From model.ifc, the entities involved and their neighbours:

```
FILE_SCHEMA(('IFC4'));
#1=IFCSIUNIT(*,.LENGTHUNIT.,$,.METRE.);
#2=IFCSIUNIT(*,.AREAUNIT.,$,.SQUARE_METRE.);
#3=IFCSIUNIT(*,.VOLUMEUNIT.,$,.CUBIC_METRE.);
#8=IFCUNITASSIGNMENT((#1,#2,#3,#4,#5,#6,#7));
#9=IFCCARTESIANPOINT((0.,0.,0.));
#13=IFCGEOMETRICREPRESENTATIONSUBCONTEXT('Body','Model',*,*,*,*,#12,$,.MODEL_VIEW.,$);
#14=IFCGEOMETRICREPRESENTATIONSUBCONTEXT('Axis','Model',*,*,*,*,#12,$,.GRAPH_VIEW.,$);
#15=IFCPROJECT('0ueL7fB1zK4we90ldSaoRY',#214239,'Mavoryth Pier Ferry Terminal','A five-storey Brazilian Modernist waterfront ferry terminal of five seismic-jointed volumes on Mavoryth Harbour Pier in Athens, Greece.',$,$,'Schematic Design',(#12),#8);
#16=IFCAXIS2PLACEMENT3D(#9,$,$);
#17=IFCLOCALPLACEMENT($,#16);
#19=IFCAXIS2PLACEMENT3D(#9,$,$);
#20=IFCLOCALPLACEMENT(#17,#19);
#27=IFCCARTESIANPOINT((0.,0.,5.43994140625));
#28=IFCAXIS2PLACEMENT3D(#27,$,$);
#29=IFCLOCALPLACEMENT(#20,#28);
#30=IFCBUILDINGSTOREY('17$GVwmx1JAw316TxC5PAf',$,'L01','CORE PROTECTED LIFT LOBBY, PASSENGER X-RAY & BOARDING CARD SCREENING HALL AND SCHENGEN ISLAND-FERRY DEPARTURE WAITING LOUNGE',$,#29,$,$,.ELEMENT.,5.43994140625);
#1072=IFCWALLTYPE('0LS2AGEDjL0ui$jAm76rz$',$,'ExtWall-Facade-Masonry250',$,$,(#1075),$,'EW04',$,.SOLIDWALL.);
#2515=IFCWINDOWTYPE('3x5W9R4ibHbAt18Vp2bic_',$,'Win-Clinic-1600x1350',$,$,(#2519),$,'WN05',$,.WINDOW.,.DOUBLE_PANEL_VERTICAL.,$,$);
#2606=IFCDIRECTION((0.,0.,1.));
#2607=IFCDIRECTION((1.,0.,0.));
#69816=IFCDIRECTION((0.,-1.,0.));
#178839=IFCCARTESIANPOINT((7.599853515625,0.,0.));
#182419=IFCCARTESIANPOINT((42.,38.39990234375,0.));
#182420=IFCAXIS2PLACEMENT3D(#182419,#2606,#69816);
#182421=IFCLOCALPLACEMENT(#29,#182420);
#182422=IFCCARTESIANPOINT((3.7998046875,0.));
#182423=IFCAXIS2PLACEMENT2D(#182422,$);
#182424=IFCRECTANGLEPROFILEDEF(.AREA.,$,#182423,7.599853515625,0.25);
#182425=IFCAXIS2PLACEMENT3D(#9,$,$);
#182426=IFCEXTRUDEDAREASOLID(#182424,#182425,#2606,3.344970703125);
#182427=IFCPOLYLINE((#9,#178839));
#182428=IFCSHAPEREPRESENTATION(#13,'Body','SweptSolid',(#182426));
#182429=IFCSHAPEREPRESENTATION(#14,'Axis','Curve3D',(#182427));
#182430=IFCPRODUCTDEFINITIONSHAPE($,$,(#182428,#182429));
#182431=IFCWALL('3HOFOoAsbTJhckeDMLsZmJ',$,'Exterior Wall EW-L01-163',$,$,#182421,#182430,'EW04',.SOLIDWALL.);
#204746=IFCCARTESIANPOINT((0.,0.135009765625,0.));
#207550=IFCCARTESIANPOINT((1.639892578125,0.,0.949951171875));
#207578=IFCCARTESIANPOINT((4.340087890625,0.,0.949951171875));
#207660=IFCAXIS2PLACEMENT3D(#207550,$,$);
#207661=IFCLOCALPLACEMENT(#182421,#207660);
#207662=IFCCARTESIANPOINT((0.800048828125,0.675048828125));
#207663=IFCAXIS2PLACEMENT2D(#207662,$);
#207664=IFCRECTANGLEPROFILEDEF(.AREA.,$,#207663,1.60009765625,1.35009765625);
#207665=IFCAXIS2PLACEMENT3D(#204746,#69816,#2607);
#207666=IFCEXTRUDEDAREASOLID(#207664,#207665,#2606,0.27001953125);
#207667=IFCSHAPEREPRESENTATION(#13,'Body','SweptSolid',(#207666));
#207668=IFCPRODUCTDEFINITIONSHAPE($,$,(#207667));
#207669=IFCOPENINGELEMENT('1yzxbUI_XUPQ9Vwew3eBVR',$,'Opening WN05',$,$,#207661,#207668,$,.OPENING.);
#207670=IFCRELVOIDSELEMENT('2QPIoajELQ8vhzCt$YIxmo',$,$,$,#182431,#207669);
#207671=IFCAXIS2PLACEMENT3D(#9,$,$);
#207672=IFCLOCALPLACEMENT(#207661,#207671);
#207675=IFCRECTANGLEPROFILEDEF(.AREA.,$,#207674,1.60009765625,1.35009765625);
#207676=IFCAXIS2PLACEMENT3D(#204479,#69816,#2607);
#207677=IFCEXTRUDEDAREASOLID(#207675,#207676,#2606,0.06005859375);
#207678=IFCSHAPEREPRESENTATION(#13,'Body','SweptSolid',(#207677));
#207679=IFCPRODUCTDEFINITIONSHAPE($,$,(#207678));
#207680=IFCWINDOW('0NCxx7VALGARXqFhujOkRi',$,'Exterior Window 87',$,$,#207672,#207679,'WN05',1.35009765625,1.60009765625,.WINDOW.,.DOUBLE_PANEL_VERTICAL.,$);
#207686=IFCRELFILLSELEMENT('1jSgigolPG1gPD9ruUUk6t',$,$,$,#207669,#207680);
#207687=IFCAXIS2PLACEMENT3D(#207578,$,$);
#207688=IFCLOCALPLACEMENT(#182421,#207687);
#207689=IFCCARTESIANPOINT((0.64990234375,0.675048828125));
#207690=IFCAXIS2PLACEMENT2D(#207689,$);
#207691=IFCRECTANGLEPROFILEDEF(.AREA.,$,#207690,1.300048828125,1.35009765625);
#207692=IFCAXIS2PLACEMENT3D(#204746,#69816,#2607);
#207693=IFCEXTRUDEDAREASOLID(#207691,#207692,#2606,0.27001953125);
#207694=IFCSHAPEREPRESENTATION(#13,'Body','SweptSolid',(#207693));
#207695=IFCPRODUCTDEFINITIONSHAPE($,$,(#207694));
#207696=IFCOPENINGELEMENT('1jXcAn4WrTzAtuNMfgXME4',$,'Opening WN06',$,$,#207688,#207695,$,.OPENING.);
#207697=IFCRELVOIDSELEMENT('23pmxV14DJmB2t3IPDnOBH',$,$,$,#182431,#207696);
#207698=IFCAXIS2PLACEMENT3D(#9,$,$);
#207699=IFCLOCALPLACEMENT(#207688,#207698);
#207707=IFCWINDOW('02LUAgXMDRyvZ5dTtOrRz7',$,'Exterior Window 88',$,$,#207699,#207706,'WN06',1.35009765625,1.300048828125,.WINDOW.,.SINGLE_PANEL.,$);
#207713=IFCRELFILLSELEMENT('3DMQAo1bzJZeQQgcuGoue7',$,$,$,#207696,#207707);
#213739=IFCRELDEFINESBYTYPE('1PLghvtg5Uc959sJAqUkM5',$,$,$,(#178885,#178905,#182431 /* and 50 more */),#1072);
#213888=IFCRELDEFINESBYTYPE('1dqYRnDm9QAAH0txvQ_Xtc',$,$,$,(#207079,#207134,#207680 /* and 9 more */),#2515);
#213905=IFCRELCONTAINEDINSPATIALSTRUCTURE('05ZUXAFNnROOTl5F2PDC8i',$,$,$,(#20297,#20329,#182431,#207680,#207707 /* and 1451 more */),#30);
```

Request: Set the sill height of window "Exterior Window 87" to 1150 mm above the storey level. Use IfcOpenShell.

```python
import numpy as np
import ifcopenshell
import ifcopenshell.api.geometry
import ifcopenshell.geom
import ifcopenshell.util.element
import ifcopenshell.util.placement
import ifcopenshell.util.shape
import ifcopenshell.util.unit

model = ifcopenshell.open("model.ifc")
unit_scale = ifcopenshell.util.unit.calculate_unit_scale(model)

window = model.by_id(207680)
opening = window.FillsVoids[0].RelatingOpeningElement
storey = ifcopenshell.util.element.get_container(window, ifc_class="IfcBuildingStorey")
level = ifcopenshell.util.placement.get_local_placement(storey.ObjectPlacement)[2, 3]

# The opening's origin need not be at the sill, so measure its lowest point.
shape = ifcopenshell.geom.create_shape(ifcopenshell.geom.settings(), opening)
bottom = ifcopenshell.util.shape.get_shape_bottom_elevation(shape, shape.geometry) / unit_scale
dz = level + 1.15 / unit_scale - bottom

shift = np.array([0.0, 0.0, dz])
# The window is placed relative to its opening, so it follows when the opening moves.
matrix = ifcopenshell.util.placement.get_local_placement(opening.ObjectPlacement)
matrix[:3, 3] += shift
ifcopenshell.api.geometry.edit_object_placement(
    model, product=opening, matrix=matrix, is_si=False, should_transform_children=True
)

print(f"moved by {dz * unit_scale:+.3f} m")

model.write("model-out.ifc")
```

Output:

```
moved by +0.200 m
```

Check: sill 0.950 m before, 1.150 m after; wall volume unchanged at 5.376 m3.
